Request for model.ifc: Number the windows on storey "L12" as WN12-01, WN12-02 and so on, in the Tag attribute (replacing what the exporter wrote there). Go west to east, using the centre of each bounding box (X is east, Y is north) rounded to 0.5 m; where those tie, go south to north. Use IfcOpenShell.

First a look at what the model holds.

```python
import ifcopenshell
import ifcopenshell.util.element
import ifcopenshell.util.placement

model = ifcopenshell.open("model.ifc")
print(model.schema)
storey = next(s for s in model.by_type("IfcBuildingStorey") if s.Name == "L12")
windows = [e for e in ifcopenshell.util.element.get_decomposition(storey) if e.is_a("IfcWindow")]
for e in sorted(windows, key=lambda e: e.id()):
    origin = ifcopenshell.util.placement.get_local_placement(e.ObjectPlacement)[:3, 3]
    print(e.id(), e.Tag, e.Name, origin.round(2) + 0.0, sep=" | ")
```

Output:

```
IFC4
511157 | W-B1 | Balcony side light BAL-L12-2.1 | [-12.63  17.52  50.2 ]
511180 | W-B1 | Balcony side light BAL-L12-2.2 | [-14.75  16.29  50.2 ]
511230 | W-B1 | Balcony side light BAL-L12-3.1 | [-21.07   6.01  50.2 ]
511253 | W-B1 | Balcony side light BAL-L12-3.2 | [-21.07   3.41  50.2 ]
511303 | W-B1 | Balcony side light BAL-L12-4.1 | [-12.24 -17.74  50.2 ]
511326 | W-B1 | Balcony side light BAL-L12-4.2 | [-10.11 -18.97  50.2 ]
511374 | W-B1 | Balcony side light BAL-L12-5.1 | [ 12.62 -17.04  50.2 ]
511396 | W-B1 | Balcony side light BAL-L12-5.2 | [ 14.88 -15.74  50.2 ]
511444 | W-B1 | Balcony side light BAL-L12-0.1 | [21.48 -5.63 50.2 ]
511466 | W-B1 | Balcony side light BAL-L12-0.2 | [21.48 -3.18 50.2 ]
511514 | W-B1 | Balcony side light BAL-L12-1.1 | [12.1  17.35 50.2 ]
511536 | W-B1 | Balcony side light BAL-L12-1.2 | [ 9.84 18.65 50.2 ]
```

```python
import ifcopenshell
import ifcopenshell.geom
import ifcopenshell.util.element
import ifcopenshell.util.shape

model = ifcopenshell.open("model.ifc")
settings = ifcopenshell.geom.settings()
settings.set("use-world-coords", True)


def centre(element):
    shape = ifcopenshell.geom.create_shape(settings, element)
    return ifcopenshell.util.shape.get_bbox_centroid(shape.geometry)


storey = next(s for s in model.by_type("IfcBuildingStorey") if s.Name == "L12")
windows = [e for e in ifcopenshell.util.element.get_decomposition(storey) if e.is_a("IfcWindow")]

# Insertion points can sit at a corner or the storey origin, so sort by the geometry (in metres).
centres = {e: centre(e) for e in windows}
windows.sort(key=lambda e: (round(centres[e][0] / 0.5), centres[e][1]))

for i, e in enumerate(windows, start=1):
    number = f"WN12-{i:02d}"
    e.Tag = number
    print(e.id(), number)

model.write("model-out.ifc")
```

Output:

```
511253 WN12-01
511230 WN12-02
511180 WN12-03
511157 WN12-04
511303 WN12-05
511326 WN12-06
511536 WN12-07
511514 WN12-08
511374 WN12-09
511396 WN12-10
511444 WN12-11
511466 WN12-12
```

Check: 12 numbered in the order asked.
